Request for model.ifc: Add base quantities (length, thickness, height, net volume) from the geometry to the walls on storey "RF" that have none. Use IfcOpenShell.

First a look at what the model holds.

```python
import ifcopenshell
import ifcopenshell.util.element
import ifcopenshell.util.unit

model = ifcopenshell.open("model.ifc")
print(model.schema)
for unit_type in ("LENGTHUNIT", "AREAUNIT", "VOLUMEUNIT"):
    print(unit_type, ifcopenshell.util.unit.calculate_unit_scale(model, unit_type))
storey = next(s for s in model.by_type("IfcBuildingStorey") if s.Name == "RF")
walls = [e for e in ifcopenshell.util.element.get_decomposition(storey) if e.is_a("IfcWall")]
for e in sorted(walls, key=lambda e: e.id()):
    print(e.id(), e.is_a(), e.Name, list(ifcopenshell.util.element.get_psets(e, qtos_only=True)), sep=" | ")
```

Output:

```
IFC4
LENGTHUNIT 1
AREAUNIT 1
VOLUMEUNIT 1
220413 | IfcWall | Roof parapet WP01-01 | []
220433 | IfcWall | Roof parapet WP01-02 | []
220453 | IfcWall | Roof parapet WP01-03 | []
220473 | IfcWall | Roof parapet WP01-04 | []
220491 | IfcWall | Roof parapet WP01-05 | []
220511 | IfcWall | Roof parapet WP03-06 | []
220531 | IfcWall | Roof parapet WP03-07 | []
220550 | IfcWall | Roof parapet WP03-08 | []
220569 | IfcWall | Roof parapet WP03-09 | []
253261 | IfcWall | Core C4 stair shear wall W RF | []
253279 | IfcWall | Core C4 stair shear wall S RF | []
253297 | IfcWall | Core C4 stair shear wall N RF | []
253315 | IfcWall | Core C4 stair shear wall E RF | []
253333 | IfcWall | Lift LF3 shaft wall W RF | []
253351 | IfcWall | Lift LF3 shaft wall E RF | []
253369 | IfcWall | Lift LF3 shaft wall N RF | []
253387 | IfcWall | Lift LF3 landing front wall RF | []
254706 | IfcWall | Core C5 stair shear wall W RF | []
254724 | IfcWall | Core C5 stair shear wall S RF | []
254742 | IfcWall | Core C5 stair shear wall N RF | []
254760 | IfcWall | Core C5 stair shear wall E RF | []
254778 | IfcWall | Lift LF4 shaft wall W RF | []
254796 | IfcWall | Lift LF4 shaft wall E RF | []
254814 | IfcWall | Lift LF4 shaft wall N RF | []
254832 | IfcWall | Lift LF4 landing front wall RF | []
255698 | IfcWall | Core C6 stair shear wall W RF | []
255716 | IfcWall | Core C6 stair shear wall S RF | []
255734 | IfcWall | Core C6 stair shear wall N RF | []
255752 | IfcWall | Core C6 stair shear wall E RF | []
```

```python
import ifcopenshell
import ifcopenshell.api.pset
import ifcopenshell.geom
import ifcopenshell.util.element
import ifcopenshell.util.shape
import ifcopenshell.util.unit

model = ifcopenshell.open("model.ifc")
unit_scale = ifcopenshell.util.unit.calculate_unit_scale(model)
volume_scale = ifcopenshell.util.unit.calculate_unit_scale(model, "VOLUMEUNIT")
settings = ifcopenshell.geom.settings()

storey = next(s for s in model.by_type("IfcBuildingStorey") if s.Name == "RF")
walls = [e for e in ifcopenshell.util.element.get_decomposition(storey) if e.is_a("IfcWall")]

for e in sorted(walls, key=lambda e: e.id()):
    if ifcopenshell.util.element.get_psets(e, qtos_only=True, should_inherit=False):
        continue
    # Geometry comes back in metres, in the element's own axes.
    shape = ifcopenshell.geom.create_shape(settings, e)
    values = {
        "Length": ifcopenshell.util.shape.get_x(shape.geometry) / unit_scale,
        "Width": ifcopenshell.util.shape.get_y(shape.geometry) / unit_scale,
        "Height": ifcopenshell.util.shape.get_z(shape.geometry) / unit_scale,
        "NetVolume": ifcopenshell.util.shape.get_volume(shape.geometry) / volume_scale,
    }
    qto = ifcopenshell.api.pset.add_qto(model, product=e, name="Qto_WallBaseQuantities")
    ifcopenshell.api.pset.edit_qto(model, qto=qto, properties=values)
    print(e.id(), {k: round(v, 3) for k, v in values.items()})

model.write("model_updated.ifc")
```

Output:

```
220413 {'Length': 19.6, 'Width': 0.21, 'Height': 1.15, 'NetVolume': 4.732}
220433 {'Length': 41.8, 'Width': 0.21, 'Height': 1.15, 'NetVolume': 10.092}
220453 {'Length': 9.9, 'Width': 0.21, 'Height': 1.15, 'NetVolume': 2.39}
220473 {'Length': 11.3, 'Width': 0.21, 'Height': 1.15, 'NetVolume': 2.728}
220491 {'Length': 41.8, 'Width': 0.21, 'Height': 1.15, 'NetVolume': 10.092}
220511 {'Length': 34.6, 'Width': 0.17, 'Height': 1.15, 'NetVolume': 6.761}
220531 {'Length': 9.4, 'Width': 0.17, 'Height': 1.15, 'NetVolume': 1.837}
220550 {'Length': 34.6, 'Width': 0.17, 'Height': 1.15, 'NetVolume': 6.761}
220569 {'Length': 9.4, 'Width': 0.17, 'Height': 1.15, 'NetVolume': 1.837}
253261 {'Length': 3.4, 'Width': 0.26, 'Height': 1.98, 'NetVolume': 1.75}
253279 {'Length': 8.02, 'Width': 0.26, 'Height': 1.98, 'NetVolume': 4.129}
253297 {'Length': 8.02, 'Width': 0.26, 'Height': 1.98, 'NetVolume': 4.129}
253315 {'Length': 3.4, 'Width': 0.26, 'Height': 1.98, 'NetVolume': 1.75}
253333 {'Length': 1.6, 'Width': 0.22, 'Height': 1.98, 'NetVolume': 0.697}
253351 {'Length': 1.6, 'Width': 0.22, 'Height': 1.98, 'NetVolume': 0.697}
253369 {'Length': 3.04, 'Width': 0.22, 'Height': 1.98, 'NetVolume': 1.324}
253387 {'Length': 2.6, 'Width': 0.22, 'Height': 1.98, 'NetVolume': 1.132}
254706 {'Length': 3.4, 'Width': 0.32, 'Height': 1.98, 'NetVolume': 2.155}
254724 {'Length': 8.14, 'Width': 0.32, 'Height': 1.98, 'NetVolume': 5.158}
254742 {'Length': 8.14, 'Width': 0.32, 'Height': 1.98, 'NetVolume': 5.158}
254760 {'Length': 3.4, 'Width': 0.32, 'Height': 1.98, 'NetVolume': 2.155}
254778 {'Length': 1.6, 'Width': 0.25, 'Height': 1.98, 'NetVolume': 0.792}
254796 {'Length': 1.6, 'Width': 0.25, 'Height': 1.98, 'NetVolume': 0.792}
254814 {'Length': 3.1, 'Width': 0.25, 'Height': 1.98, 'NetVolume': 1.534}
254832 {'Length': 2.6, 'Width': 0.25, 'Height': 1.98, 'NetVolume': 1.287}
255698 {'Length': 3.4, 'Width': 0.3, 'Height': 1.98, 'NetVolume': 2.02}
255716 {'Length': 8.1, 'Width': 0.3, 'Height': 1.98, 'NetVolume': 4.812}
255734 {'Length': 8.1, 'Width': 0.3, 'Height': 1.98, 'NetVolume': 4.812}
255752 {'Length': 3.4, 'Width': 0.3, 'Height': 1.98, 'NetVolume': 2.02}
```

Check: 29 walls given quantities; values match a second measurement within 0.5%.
